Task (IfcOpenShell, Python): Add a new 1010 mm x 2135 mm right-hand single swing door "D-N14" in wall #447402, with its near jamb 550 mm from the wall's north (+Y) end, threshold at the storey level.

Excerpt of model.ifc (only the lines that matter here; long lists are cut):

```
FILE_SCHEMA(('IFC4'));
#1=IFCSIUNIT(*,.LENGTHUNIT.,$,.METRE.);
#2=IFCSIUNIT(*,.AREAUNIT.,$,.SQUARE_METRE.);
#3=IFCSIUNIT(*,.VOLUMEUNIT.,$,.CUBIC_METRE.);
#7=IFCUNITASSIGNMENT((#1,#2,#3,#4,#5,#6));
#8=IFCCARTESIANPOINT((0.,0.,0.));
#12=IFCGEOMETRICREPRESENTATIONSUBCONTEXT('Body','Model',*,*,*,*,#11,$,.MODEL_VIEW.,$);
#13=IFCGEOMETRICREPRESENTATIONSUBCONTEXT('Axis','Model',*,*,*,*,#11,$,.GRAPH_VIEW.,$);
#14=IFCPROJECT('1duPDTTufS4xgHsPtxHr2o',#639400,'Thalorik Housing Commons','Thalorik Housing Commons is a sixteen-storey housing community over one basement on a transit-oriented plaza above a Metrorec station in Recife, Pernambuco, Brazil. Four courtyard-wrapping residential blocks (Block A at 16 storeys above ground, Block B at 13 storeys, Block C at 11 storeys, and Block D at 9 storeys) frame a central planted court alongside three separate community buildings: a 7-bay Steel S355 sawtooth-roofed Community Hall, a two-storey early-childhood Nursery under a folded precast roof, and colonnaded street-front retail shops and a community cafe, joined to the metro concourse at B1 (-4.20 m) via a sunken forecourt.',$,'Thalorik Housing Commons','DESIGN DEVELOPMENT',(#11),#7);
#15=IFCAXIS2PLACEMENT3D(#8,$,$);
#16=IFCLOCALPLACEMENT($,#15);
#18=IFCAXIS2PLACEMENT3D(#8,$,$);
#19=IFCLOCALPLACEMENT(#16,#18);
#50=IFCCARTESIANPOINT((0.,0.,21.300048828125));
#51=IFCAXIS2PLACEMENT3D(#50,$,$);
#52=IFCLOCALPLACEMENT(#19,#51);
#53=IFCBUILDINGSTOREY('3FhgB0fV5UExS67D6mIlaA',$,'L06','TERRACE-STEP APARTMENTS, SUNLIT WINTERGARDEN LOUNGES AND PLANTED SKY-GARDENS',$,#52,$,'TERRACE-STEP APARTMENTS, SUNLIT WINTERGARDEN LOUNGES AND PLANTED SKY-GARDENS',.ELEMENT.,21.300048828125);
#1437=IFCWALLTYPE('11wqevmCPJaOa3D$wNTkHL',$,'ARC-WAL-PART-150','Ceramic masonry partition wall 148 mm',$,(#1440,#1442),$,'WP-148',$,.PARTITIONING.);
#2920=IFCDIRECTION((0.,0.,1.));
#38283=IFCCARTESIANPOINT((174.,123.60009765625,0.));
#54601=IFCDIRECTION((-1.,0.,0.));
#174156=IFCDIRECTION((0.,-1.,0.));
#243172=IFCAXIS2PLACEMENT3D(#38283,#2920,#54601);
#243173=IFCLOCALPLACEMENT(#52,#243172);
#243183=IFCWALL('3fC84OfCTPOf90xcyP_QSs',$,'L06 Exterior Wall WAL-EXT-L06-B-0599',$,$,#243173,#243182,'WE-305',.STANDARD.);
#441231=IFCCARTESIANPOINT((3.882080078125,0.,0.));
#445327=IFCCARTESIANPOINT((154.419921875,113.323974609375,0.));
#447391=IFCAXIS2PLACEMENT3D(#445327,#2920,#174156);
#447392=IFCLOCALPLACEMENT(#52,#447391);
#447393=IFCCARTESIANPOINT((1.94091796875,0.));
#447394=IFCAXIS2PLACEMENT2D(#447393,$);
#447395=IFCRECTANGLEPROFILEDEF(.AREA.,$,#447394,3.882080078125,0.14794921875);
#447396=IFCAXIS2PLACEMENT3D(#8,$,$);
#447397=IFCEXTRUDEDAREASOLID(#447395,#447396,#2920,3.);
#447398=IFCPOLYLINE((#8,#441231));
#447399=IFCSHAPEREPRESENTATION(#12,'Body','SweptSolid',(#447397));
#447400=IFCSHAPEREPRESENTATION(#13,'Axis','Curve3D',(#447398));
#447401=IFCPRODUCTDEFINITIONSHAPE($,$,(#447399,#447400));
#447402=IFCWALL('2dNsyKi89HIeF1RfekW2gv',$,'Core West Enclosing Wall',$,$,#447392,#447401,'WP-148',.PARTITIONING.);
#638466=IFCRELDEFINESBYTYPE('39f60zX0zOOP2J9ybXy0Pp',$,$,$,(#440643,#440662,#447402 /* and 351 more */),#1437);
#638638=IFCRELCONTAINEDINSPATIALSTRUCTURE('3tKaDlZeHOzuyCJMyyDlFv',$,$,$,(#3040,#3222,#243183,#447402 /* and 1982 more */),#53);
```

```python
import numpy as np
import ifcopenshell
import ifcopenshell.api.feature
import ifcopenshell.api.geometry
import ifcopenshell.api.root
import ifcopenshell.api.spatial
import ifcopenshell.geom
import ifcopenshell.util.element
import ifcopenshell.util.placement
import ifcopenshell.util.representation
import ifcopenshell.util.shape
import ifcopenshell.util.unit

model = ifcopenshell.open("model.ifc")
unit_scale = ifcopenshell.util.unit.calculate_unit_scale(model)
settings = ifcopenshell.geom.settings()


def volume(element):
    """Net volume in cubic metres, openings subtracted."""
    shape = ifcopenshell.geom.create_shape(settings, element)
    return ifcopenshell.util.shape.get_volume(shape.geometry)


wall = model.by_guid("2dNsyKi89HIeF1RfekW2gv")
storey = ifcopenshell.util.element.get_container(wall, ifc_class="IfcBuildingStorey")
context = ifcopenshell.util.representation.get_context(model, "Model", "Body", "MODEL_VIEW")
before = volume(wall)

width, height, from_end, sill = 1.01, 2.135, 0.55, 0.0  # metres

# The wall runs along its own X axis, and the end named is its -X end.
wall_shape = ifcopenshell.geom.create_shape(settings, wall)
x, y, z = ifcopenshell.util.shape.get_vertices(wall_shape.geometry).T
start = x.min() + from_end
face, thickness = float(y.min()), float(y.max() - y.min())
wall_matrix = ifcopenshell.util.placement.get_local_placement(wall.ObjectPlacement)
level = ifcopenshell.util.placement.get_local_placement(storey.ObjectPlacement)[2, 3]


def in_wall(x, y):
    """Placement at x, y metres in the wall's axes, at sill height."""
    matrix = wall_matrix.copy()
    matrix[:, 3] = wall_matrix @ np.array([x / unit_scale, y / unit_scale, 0.0, 1.0])
    matrix[2, 3] = level + sill / unit_scale
    return matrix


# Opening: a box that overshoots both wall faces by 50 mm.
opening = ifcopenshell.api.root.create_entity(model, ifc_class="IfcOpeningElement", predefined_type="OPENING")
box = ifcopenshell.api.geometry.add_wall_representation(
    model, context=context, length=width, height=height, thickness=thickness + 0.1
)
ifcopenshell.api.geometry.assign_representation(model, product=opening, representation=box)
ifcopenshell.api.geometry.edit_object_placement(model, product=opening, matrix=in_wall(start, face - 0.05), is_si=False)
ifcopenshell.api.feature.add_feature(model, feature=opening, element=wall)

door = ifcopenshell.api.root.create_entity(model, ifc_class="IfcDoor", name="D-N14", predefined_type="DOOR")
door.OverallWidth, door.OverallHeight = width / unit_scale, height / unit_scale
door.OperationType = "SINGLE_SWING_RIGHT"
body = ifcopenshell.api.geometry.add_door_representation(
    model,
    context=context,
    overall_width=door.OverallWidth,
    overall_height=door.OverallHeight,
    operation_type="SINGLE_SWING_RIGHT",
    lining_properties={"LiningDepth": thickness / unit_scale, "ThresholdDepth": thickness / unit_scale},
)
ifcopenshell.api.geometry.assign_representation(model, product=door, representation=body)
ifcopenshell.api.spatial.assign_container(model, products=[door], relating_structure=storey)
ifcopenshell.api.feature.add_filling(model, opening=opening, element=door)

# The lining spans the wall, so the door starts at the wall face.
ifcopenshell.api.geometry.edit_object_placement(model, product=door, matrix=in_wall(start, face), is_si=False)

after = volume(wall)

print(f"wall volume {before:.3f} -> {after:.3f} m3")

model.write("model_v2.ifc")
```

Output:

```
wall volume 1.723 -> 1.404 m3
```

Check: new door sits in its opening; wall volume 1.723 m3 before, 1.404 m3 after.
